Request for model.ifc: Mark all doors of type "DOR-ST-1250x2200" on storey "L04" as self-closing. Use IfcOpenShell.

First a look at what the model holds.

```python
import ifcopenshell
import ifcopenshell.util.element

model = ifcopenshell.open("model.ifc")
print(model.schema)
storey = next(s for s in model.by_type("IfcBuildingStorey") if s.Name == "L04")
doors = [e for e in ifcopenshell.util.element.get_decomposition(storey) if e.is_a("IfcDoor")]
seen = {}
for e in doors:
    element_type = ifcopenshell.util.element.get_type(e)
    key = (element_type.Name if element_type != e and element_type else None, ifcopenshell.util.element.get_pset(e, "Pset_DoorCommon", "SelfClosing"))
    seen[key] = seen.get(key, 0) + 1
for (name, value), count in sorted(seen.items(), key=str):
    print(count, "x", name, "|", value)
```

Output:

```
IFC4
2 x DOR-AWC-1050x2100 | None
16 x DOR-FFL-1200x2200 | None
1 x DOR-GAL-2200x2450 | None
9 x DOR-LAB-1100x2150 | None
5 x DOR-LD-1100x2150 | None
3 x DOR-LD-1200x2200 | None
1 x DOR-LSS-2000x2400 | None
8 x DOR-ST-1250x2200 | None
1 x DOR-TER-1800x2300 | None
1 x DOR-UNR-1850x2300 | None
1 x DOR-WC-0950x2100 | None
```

```python
import ifcopenshell
import ifcopenshell.api.pset
import ifcopenshell.util.element

model = ifcopenshell.open("model.ifc")

storey = next(s for s in model.by_type("IfcBuildingStorey") if s.Name == "L04")
doors = [e for e in ifcopenshell.util.element.get_decomposition(storey) if e.is_a("IfcDoor")]

count = 0
for e in doors:
    element_type = ifcopenshell.util.element.get_type(e)
    if element_type in (None, e) or element_type.Name != "DOR-ST-1250x2200":
        continue
    # add_pset returns the element's existing set when there is one.
    pset = ifcopenshell.api.pset.add_pset(model, product=e, name="Pset_DoorCommon")
    ifcopenshell.api.pset.edit_pset(model, pset=pset, properties={"SelfClosing": True})
    count += 1

print(count, "doors updated")

model.write("model-out.ifc")
```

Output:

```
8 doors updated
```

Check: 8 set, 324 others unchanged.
